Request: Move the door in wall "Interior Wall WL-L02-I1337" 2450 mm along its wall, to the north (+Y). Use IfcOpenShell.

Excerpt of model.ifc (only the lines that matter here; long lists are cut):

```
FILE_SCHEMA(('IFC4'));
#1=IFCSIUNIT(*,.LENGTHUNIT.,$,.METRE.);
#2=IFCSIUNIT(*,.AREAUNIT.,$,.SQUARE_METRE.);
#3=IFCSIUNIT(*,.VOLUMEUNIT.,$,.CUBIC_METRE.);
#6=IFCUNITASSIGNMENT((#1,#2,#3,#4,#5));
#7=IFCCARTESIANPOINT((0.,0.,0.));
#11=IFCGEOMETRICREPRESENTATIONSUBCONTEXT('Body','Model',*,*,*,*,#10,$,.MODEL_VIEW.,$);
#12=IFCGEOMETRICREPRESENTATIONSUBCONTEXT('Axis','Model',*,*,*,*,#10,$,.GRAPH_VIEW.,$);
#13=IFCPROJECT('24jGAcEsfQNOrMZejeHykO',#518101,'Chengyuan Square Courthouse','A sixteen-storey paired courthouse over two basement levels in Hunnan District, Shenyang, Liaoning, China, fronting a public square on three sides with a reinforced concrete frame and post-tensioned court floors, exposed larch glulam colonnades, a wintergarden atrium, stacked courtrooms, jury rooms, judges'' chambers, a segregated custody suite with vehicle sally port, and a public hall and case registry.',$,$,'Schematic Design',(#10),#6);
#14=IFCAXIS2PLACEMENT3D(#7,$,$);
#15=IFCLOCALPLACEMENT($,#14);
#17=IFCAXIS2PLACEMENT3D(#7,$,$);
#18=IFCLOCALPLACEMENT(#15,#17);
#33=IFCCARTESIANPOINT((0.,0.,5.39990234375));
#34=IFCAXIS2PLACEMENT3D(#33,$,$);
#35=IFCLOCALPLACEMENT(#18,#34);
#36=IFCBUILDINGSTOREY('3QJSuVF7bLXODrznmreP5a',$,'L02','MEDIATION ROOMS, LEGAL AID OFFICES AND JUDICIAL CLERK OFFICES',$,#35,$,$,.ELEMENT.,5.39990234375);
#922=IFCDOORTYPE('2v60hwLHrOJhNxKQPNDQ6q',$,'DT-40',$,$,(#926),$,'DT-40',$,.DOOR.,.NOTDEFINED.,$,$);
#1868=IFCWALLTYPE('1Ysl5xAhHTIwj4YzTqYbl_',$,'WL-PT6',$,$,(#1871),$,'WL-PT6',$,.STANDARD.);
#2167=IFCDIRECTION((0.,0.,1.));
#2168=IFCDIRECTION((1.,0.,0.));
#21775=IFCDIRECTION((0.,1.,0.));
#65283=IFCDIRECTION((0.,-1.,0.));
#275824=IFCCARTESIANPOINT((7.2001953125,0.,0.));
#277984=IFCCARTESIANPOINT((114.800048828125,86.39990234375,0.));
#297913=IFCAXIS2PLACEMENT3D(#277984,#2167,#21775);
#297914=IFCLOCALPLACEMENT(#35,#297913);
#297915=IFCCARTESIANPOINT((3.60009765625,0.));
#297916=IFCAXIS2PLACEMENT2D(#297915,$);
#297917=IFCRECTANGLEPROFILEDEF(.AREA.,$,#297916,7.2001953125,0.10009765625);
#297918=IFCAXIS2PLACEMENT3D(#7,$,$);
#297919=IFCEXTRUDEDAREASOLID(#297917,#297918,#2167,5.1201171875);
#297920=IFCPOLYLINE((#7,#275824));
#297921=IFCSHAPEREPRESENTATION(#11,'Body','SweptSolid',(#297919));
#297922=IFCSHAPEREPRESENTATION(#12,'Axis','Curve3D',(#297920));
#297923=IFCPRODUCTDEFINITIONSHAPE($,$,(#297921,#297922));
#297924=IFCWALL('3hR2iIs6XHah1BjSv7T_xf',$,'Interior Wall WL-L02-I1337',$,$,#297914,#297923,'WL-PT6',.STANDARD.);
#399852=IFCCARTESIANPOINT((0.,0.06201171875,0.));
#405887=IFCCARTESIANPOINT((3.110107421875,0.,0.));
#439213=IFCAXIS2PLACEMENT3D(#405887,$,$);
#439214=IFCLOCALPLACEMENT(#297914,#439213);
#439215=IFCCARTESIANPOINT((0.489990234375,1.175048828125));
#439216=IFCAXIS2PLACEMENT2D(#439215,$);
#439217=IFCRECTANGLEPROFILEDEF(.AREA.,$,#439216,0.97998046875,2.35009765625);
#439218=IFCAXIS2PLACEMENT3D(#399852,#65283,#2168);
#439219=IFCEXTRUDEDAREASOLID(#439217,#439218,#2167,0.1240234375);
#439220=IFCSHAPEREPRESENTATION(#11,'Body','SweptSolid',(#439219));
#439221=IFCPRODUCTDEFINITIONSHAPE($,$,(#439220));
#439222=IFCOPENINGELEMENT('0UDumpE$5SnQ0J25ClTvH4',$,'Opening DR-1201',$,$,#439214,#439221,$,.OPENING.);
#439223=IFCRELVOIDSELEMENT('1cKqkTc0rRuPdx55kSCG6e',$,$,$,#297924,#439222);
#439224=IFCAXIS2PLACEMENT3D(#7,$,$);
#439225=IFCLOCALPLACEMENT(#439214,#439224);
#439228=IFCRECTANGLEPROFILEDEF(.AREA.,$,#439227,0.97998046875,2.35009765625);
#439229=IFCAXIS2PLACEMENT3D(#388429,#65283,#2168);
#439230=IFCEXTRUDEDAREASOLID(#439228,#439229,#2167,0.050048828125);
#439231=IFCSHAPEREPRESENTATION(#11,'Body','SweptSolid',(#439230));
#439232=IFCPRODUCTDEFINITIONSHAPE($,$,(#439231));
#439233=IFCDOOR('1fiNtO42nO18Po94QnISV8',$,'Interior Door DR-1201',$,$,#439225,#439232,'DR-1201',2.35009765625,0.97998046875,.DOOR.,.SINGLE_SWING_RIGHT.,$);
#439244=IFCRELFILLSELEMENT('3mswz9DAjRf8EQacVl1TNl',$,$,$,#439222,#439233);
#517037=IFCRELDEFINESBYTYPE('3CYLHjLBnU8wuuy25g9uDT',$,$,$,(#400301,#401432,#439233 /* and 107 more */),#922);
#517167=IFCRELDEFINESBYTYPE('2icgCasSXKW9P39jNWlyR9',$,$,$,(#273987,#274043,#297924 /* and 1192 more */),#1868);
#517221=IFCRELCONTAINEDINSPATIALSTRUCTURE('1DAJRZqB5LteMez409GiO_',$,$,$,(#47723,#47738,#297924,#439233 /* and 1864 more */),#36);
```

```python
import ifcopenshell
import ifcopenshell.api.geometry
import ifcopenshell.util.placement
import ifcopenshell.util.unit

model = ifcopenshell.open("model.ifc")
unit_scale = ifcopenshell.util.unit.calculate_unit_scale(model)

door = model.by_guid("1fiNtO42nO18Po94QnISV8")
opening = door.FillsVoids[0].RelatingOpeningElement
wall = opening.VoidsElements[0].RelatingBuildingElement

wall_matrix = ifcopenshell.util.placement.get_local_placement(wall.ObjectPlacement)
shift = wall_matrix[:3, 0] * 2.45 / unit_scale
before = ifcopenshell.util.placement.get_local_placement(door.ObjectPlacement)[:3, 3].copy()

# The door is placed relative to its opening, so it follows when the opening moves.
matrix = ifcopenshell.util.placement.get_local_placement(opening.ObjectPlacement)
matrix[:3, 3] += shift
ifcopenshell.api.geometry.edit_object_placement(
    model, product=opening, matrix=matrix, is_si=False, should_transform_children=True
)

after = ifcopenshell.util.placement.get_local_placement(door.ObjectPlacement)[:3, 3]
print("door moved by", (after - before).round(3) + 0.0)

model.write("model_updated.ifc")
```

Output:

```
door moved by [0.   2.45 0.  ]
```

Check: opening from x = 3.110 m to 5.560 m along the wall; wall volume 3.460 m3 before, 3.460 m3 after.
